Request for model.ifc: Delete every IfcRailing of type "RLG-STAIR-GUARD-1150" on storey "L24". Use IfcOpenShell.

First a look at what the model holds.

```python
import ifcopenshell
import ifcopenshell.util.element

model = ifcopenshell.open("model.ifc")
print(model.schema)
storey = next(s for s in model.by_type("IfcBuildingStorey") if s.Name == "L24")
railings = [e for e in ifcopenshell.util.element.get_decomposition(storey) if e.is_a("IfcRailing")]
seen = {}
for e in railings:
    element_type = ifcopenshell.util.element.get_type(e)
    name = element_type.Name if element_type not in (None, e) else None
    seen[name] = seen.get(name, 0) + 1
for name, count in sorted(seen.items(), key=str):
    print(count, "x", name)
```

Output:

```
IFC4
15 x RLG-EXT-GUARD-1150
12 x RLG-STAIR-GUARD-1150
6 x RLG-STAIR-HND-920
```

```python
import ifcopenshell
import ifcopenshell.api.root
import ifcopenshell.util.element

model = ifcopenshell.open("model.ifc")

storey = next(s for s in model.by_type("IfcBuildingStorey") if s.Name == "L24")
railings = [e for e in ifcopenshell.util.element.get_decomposition(storey) if e.is_a("IfcRailing")]
targets = [e for e in railings if (t := ifcopenshell.util.element.get_type(e)) not in (None, e) and t.Name == "RLG-STAIR-GUARD-1150"]

for e in targets:
    ifcopenshell.api.root.remove_product(model, product=e)
print(len(targets), "removed")

model.write("model-out.ifc")
```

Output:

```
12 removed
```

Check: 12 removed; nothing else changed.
